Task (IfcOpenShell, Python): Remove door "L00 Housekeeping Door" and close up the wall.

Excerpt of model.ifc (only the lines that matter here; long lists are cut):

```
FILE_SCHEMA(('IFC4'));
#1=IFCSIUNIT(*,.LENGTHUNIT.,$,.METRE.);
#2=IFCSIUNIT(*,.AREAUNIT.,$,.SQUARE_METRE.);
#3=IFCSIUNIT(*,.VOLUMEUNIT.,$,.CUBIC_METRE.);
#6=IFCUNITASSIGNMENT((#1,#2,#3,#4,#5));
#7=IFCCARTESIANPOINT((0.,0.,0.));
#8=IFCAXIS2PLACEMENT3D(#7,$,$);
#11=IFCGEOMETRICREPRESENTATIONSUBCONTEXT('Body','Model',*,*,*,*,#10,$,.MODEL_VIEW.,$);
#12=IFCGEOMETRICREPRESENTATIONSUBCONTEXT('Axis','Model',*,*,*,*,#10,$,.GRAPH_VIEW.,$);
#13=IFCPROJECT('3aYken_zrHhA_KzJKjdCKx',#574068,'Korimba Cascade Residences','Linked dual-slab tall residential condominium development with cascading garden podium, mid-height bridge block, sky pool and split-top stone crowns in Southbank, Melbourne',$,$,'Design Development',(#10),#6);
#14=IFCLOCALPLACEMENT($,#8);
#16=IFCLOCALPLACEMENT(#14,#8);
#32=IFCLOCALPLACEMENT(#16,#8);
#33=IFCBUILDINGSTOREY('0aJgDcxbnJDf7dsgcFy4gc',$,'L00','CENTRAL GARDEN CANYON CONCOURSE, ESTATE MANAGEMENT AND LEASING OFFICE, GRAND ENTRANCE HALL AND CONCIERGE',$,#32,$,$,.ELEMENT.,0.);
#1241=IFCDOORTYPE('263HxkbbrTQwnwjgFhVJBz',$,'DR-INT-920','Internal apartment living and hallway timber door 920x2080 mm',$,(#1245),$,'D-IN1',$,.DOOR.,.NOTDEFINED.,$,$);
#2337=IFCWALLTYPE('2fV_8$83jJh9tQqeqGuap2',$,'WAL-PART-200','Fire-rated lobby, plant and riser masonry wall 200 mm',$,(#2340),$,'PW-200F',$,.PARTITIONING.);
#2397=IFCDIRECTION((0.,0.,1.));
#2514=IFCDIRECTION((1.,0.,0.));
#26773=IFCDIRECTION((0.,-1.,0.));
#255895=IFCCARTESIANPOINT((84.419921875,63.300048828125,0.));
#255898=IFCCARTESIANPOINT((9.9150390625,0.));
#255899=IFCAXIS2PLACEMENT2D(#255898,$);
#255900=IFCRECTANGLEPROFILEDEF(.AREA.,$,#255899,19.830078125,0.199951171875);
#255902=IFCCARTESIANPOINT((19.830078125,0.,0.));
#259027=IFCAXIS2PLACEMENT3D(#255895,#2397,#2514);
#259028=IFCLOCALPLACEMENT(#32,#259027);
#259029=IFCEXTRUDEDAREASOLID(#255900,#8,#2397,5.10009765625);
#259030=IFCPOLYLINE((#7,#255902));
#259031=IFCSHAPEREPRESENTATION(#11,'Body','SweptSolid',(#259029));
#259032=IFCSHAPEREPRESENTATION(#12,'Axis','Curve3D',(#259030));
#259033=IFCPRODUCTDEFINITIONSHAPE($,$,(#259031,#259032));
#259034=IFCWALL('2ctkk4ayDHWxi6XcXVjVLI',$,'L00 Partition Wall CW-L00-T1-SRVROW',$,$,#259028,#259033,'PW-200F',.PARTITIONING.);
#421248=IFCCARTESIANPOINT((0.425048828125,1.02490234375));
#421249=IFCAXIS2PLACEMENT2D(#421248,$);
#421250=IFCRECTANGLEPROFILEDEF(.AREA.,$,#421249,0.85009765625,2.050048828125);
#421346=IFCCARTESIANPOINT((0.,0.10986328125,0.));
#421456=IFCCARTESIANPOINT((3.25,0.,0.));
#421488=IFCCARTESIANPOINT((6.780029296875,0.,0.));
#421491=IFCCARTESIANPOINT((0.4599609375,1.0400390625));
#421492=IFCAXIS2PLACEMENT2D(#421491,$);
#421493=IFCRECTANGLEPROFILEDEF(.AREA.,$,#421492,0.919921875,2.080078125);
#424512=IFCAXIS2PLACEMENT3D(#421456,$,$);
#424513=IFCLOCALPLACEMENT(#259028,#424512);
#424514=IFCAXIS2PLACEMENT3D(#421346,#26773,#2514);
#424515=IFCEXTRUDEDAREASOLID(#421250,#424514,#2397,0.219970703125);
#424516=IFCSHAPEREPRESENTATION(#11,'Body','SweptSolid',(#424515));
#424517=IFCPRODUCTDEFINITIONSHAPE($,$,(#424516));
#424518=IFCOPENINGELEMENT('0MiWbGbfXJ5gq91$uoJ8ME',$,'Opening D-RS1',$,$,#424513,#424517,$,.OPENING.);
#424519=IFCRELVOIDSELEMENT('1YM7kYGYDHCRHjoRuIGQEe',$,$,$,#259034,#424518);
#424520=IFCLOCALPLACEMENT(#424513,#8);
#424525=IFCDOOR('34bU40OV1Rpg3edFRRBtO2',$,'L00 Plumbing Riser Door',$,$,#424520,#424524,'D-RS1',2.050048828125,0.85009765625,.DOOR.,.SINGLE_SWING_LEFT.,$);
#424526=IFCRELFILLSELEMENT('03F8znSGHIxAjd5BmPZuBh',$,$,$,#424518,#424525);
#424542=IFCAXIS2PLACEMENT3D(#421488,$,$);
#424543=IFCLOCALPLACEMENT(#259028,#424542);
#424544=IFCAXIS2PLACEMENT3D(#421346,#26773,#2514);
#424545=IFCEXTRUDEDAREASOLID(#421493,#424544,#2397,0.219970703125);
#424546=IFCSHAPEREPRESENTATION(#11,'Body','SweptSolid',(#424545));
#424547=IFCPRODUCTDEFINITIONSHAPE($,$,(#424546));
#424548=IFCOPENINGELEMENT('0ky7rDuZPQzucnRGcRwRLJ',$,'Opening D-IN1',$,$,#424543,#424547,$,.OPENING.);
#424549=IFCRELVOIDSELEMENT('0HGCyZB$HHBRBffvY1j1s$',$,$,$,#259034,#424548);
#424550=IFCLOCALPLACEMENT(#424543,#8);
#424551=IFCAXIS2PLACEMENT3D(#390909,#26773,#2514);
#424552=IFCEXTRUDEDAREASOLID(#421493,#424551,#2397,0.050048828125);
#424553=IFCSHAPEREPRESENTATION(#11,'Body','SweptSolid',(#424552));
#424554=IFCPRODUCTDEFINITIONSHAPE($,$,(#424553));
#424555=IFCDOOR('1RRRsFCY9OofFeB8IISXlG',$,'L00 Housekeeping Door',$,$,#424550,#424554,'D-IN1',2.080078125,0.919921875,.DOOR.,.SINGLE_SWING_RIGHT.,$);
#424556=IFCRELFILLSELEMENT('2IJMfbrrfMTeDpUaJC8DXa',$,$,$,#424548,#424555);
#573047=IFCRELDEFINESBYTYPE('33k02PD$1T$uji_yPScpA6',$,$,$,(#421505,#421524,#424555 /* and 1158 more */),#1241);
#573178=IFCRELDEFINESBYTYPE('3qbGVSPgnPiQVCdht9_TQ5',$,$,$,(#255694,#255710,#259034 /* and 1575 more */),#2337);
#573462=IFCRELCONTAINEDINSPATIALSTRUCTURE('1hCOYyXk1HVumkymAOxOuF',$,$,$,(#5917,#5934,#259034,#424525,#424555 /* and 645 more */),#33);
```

```python
import ifcopenshell
import ifcopenshell.api.feature
import ifcopenshell.api.root
import ifcopenshell.geom
import ifcopenshell.util.shape

model = ifcopenshell.open("model.ifc")
settings = ifcopenshell.geom.settings()


def volume(element):
    """Net volume in cubic metres, openings subtracted."""
    shape = ifcopenshell.geom.create_shape(settings, element)
    return ifcopenshell.util.shape.get_volume(shape.geometry)


door = model.by_id(424555)
opening = door.FillsVoids[0].RelatingOpeningElement
wall = opening.VoidsElements[0].RelatingBuildingElement
before = volume(wall)

ifcopenshell.api.root.remove_product(model, product=door)
ifcopenshell.api.feature.remove_feature(model, feature=opening)

after = volume(wall)

print(f"wall volume {before:.3f} -> {after:.3f} m3")

model.write("model_updated.ifc")
```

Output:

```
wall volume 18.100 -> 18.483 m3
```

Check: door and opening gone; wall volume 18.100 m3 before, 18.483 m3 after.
